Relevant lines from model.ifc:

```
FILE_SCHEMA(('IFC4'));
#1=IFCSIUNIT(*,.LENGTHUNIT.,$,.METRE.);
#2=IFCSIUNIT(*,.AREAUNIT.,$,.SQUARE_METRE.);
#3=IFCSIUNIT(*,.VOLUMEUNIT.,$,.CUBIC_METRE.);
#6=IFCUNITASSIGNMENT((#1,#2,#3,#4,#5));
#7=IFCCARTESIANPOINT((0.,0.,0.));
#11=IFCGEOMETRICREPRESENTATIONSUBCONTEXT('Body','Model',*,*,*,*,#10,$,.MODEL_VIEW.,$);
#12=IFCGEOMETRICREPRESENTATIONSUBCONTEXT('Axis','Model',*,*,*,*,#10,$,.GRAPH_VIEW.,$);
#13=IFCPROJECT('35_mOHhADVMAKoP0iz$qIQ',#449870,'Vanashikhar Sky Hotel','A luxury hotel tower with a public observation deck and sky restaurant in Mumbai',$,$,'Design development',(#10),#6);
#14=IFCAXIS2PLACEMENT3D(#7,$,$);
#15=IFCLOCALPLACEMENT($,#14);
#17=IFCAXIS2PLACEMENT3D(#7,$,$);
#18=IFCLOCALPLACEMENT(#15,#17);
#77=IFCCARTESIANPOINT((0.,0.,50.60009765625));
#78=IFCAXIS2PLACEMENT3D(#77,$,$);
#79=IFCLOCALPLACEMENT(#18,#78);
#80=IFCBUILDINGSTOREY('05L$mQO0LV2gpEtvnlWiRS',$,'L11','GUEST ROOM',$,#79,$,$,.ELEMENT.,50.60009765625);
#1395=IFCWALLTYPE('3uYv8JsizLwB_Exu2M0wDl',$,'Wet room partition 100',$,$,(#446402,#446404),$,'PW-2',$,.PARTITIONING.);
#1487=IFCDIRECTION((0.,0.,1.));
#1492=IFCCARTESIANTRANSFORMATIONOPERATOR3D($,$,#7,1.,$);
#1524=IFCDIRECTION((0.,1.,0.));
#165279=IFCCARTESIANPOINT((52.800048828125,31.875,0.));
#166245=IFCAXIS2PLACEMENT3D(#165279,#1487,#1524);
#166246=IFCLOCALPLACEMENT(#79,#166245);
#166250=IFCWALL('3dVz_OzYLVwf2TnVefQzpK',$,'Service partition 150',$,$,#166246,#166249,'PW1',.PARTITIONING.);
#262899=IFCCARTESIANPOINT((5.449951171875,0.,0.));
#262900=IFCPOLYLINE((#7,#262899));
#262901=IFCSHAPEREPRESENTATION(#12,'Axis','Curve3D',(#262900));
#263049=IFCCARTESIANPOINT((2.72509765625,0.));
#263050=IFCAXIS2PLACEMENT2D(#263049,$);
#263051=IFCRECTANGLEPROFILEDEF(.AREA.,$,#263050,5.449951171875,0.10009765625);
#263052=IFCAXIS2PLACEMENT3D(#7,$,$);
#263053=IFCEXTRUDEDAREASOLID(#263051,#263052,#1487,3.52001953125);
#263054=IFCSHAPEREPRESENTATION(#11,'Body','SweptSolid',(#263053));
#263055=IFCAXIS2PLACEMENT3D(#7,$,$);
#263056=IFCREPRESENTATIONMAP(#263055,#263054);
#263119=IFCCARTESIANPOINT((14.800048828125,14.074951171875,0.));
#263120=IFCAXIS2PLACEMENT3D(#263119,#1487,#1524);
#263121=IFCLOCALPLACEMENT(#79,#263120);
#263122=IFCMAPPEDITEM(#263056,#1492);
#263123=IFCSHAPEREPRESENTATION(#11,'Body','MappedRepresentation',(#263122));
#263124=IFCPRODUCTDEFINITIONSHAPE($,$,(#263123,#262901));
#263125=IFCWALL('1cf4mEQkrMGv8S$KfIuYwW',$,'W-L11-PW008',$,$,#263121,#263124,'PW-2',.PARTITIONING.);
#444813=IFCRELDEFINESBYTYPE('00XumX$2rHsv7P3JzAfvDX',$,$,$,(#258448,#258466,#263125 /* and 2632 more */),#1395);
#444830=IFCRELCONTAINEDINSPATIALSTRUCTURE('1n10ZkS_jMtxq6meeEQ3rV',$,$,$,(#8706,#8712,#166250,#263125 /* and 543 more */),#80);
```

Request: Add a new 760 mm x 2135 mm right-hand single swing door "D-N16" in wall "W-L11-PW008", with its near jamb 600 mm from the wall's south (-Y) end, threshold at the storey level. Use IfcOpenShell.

```python
import numpy as np
import ifcopenshell
import ifcopenshell.api.feature
import ifcopenshell.api.geometry
import ifcopenshell.api.root
import ifcopenshell.api.spatial
import ifcopenshell.geom
import ifcopenshell.util.element
import ifcopenshell.util.placement
import ifcopenshell.util.representation
import ifcopenshell.util.shape
import ifcopenshell.util.unit

model = ifcopenshell.open("model.ifc")
unit_scale = ifcopenshell.util.unit.calculate_unit_scale(model)
settings = ifcopenshell.geom.settings()


def volume(element):
    """Net volume in cubic metres, openings subtracted."""
    shape = ifcopenshell.geom.create_shape(settings, element)
    return ifcopenshell.util.shape.get_volume(shape.geometry)


wall = model.by_guid("1cf4mEQkrMGv8S$KfIuYwW")
storey = ifcopenshell.util.element.get_container(wall, ifc_class="IfcBuildingStorey")
context = ifcopenshell.util.representation.get_context(model, "Model", "Body", "MODEL_VIEW")
before = volume(wall)

width, height, from_end, sill = 0.76, 2.135, 0.6, 0.0  # metres

# The wall runs along its own X axis, and the end named is its -X end.
wall_shape = ifcopenshell.geom.create_shape(settings, wall)
x, y, z = ifcopenshell.util.shape.get_vertices(wall_shape.geometry).T
start = x.min() + from_end
face, thickness = float(y.min()), float(y.max() - y.min())
wall_matrix = ifcopenshell.util.placement.get_local_placement(wall.ObjectPlacement)
level = ifcopenshell.util.placement.get_local_placement(storey.ObjectPlacement)[2, 3]


def in_wall(x, y):
    """Placement at x, y metres in the wall's axes, at sill height."""
    matrix = wall_matrix.copy()
    matrix[:, 3] = wall_matrix @ np.array([x / unit_scale, y / unit_scale, 0.0, 1.0])
    matrix[2, 3] = level + sill / unit_scale
    return matrix


# Opening: a box that overshoots both wall faces by 50 mm.
opening = ifcopenshell.api.root.create_entity(model, ifc_class="IfcOpeningElement", predefined_type="OPENING")
box = ifcopenshell.api.geometry.add_wall_representation(
    model, context=context, length=width, height=height, thickness=thickness + 0.1
)
ifcopenshell.api.geometry.assign_representation(model, product=opening, representation=box)
ifcopenshell.api.geometry.edit_object_placement(model, product=opening, matrix=in_wall(start, face - 0.05), is_si=False)
ifcopenshell.api.feature.add_feature(model, feature=opening, element=wall)

door = ifcopenshell.api.root.create_entity(model, ifc_class="IfcDoor", name="D-N16", predefined_type="DOOR")
door.OverallWidth, door.OverallHeight = width / unit_scale, height / unit_scale
door.OperationType = "SINGLE_SWING_RIGHT"
body = ifcopenshell.api.geometry.add_door_representation(
    model,
    context=context,
    overall_width=door.OverallWidth,
    overall_height=door.OverallHeight,
    operation_type="SINGLE_SWING_RIGHT",
    lining_properties={"LiningDepth": thickness / unit_scale, "ThresholdDepth": thickness / unit_scale},
)
ifcopenshell.api.geometry.assign_representation(model, product=door, representation=body)
ifcopenshell.api.spatial.assign_container(model, products=[door], relating_structure=storey)
ifcopenshell.api.feature.add_filling(model, opening=opening, element=door)

# The lining spans the wall, so the door starts at the wall face.
ifcopenshell.api.geometry.edit_object_placement(model, product=door, matrix=in_wall(start, face), is_si=False)

after = volume(wall)

print(f"wall volume {before:.3f} -> {after:.3f} m3")

model.write("model-out.ifc")
```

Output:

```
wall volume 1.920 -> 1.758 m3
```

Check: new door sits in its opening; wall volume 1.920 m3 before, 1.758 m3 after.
